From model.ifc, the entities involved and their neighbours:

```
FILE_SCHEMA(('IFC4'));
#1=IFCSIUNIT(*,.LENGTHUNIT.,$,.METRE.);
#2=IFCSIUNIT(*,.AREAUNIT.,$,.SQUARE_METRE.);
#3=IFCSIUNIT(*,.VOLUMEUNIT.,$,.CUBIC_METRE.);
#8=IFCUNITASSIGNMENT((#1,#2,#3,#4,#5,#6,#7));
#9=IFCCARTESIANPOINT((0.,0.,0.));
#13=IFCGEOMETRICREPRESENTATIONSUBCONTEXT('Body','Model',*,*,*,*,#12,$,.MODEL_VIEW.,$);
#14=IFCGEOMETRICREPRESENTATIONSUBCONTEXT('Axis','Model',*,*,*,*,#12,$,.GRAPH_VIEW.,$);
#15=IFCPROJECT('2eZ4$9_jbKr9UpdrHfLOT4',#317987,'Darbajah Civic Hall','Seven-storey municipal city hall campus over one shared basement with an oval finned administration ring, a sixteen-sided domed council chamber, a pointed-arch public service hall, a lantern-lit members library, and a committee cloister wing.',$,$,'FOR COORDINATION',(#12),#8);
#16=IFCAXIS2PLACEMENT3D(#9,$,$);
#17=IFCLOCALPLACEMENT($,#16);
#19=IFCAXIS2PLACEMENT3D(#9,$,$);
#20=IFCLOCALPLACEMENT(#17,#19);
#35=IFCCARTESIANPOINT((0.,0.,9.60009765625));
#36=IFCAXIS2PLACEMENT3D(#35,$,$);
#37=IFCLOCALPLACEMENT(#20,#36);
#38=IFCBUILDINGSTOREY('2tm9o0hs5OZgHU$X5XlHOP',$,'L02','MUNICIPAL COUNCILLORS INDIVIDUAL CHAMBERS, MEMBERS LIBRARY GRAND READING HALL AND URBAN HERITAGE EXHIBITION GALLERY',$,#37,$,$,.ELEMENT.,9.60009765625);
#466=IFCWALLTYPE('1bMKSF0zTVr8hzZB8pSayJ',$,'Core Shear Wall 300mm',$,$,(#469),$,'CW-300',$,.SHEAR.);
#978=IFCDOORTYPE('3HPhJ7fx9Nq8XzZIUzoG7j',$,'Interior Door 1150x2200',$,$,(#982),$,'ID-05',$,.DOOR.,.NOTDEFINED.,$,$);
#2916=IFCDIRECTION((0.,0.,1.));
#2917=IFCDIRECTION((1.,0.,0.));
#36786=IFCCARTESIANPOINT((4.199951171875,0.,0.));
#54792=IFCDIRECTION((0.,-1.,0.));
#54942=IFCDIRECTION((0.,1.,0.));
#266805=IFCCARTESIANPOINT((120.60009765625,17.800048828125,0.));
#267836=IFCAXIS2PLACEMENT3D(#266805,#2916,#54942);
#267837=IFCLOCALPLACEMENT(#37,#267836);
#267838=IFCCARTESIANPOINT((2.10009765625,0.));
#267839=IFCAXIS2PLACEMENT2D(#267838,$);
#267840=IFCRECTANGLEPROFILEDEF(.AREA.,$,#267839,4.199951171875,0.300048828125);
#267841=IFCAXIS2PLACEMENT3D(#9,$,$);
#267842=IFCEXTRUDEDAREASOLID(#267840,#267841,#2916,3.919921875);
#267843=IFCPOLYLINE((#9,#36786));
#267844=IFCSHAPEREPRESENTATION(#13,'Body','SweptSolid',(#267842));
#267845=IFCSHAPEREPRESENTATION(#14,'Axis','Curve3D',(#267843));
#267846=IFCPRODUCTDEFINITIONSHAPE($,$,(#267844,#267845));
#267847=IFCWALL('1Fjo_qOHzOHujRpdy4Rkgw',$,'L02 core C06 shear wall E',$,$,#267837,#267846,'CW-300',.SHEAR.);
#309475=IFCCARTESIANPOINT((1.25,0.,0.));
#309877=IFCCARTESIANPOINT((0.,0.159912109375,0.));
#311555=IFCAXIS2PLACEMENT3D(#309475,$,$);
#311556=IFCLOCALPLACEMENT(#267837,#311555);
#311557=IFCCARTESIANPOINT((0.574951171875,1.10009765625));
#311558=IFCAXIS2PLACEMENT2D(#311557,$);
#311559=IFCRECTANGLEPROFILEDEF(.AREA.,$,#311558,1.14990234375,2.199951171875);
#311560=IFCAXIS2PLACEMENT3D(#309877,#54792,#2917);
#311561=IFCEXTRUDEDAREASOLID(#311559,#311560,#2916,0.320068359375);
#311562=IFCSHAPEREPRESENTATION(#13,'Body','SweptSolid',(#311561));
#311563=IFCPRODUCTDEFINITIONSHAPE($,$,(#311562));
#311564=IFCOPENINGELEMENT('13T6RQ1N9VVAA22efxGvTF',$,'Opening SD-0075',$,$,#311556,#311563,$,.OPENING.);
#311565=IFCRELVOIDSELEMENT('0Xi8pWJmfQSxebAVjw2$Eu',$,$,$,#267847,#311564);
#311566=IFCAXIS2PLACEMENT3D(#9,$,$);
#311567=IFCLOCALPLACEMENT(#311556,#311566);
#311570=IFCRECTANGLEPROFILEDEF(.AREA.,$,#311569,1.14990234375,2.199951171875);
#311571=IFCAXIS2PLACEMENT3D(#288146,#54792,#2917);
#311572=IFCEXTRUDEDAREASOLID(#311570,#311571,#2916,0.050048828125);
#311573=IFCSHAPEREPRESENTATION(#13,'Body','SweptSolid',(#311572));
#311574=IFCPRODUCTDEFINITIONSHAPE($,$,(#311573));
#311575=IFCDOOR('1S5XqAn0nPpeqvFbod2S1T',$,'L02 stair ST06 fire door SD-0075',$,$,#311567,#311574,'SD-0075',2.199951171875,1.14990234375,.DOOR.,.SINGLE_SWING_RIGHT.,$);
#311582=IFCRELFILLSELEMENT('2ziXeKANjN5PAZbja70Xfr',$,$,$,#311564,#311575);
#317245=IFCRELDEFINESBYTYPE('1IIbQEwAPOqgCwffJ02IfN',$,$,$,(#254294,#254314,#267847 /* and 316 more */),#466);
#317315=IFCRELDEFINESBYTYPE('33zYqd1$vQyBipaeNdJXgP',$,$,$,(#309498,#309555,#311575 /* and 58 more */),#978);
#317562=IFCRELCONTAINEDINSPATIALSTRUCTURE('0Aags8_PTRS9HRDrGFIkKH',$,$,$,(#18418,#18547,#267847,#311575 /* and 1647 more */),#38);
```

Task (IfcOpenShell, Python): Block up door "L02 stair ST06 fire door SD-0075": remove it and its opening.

```python
import ifcopenshell
import ifcopenshell.api.feature
import ifcopenshell.api.root
import ifcopenshell.geom
import ifcopenshell.util.shape

model = ifcopenshell.open("model.ifc")
settings = ifcopenshell.geom.settings()


def volume(element):
    """Net volume in cubic metres, openings subtracted."""
    shape = ifcopenshell.geom.create_shape(settings, element)
    return ifcopenshell.util.shape.get_volume(shape.geometry)


door = model.by_id(311575)
opening = door.FillsVoids[0].RelatingOpeningElement
wall = opening.VoidsElements[0].RelatingBuildingElement
before = volume(wall)

ifcopenshell.api.root.remove_product(model, product=door)
ifcopenshell.api.feature.remove_feature(model, feature=opening)

after = volume(wall)

print(f"wall volume {before:.3f} -> {after:.3f} m3")

model.write("model_rev.ifc")
```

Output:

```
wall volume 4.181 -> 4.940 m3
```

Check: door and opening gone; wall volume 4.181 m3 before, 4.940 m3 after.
